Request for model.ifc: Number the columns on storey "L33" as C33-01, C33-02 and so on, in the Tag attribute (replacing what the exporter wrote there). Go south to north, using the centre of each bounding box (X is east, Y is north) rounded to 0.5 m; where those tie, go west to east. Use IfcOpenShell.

First a look at what the model holds.

```python
import ifcopenshell
import ifcopenshell.util.element
import ifcopenshell.util.placement

model = ifcopenshell.open("model.ifc")
print(model.schema)
storey = next(s for s in model.by_type("IfcBuildingStorey") if s.Name == "L33")
columns = [e for e in ifcopenshell.util.element.get_decomposition(storey) if e.is_a("IfcColumn")]
for e in sorted(columns, key=lambda e: e.id()):
    origin = ifcopenshell.util.placement.get_local_placement(e.ObjectPlacement)[:3, 3]
    print(e.id(), e.Tag, e.Name, origin.round(2) + 0.0, sep=" | ")
```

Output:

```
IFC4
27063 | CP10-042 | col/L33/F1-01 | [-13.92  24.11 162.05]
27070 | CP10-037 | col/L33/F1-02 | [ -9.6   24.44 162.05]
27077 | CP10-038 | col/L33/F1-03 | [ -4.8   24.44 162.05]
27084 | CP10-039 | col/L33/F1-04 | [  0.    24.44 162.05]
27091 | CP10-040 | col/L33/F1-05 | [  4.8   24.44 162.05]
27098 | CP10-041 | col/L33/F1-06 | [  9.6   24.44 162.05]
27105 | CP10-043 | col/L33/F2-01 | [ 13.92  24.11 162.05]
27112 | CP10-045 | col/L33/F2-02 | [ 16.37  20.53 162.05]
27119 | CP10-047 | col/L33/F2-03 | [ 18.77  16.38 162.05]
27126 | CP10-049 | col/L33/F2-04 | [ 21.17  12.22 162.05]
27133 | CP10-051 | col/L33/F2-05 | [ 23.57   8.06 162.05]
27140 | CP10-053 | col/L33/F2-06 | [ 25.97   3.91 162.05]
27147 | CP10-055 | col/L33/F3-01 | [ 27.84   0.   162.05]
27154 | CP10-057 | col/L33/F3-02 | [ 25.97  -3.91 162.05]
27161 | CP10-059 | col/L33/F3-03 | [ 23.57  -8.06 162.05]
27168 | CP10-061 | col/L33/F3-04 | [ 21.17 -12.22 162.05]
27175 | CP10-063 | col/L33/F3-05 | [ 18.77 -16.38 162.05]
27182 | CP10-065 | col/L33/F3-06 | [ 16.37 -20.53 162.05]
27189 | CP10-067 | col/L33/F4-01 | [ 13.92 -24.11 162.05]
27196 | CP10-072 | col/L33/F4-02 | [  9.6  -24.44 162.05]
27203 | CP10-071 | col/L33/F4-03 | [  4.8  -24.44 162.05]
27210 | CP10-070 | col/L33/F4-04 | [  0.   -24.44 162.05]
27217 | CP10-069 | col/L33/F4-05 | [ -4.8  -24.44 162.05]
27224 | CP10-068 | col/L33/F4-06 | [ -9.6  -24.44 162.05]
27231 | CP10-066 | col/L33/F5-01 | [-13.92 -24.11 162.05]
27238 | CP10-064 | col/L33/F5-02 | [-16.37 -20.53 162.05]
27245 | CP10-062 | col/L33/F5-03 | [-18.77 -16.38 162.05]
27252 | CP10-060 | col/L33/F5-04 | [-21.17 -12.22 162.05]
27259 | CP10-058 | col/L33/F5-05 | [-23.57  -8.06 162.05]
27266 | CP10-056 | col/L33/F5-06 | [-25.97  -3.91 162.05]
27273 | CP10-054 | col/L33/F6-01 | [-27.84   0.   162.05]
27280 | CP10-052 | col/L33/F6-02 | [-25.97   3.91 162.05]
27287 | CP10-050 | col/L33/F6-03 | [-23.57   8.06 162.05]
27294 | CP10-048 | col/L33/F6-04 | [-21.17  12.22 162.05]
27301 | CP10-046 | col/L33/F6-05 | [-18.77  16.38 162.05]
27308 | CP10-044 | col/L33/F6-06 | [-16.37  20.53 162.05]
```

```python
import ifcopenshell
import ifcopenshell.geom
import ifcopenshell.util.element
import ifcopenshell.util.shape

model = ifcopenshell.open("model.ifc")
settings = ifcopenshell.geom.settings()
settings.set("use-world-coords", True)


def centre(element):
    shape = ifcopenshell.geom.create_shape(settings, element)
    return ifcopenshell.util.shape.get_bbox_centroid(shape.geometry)


storey = next(s for s in model.by_type("IfcBuildingStorey") if s.Name == "L33")
columns = [e for e in ifcopenshell.util.element.get_decomposition(storey) if e.is_a("IfcColumn")]

# Insertion points can sit at a corner or the storey origin, so sort by the geometry (in metres).
centres = {e: centre(e) for e in columns}
columns.sort(key=lambda e: (round(centres[e][1] / 0.5), centres[e][0]))

for i, e in enumerate(columns, start=1):
    number = f"C33-{i:02d}"
    e.Tag = number
    print(e.id(), number)

model.write("model-out.ifc")
```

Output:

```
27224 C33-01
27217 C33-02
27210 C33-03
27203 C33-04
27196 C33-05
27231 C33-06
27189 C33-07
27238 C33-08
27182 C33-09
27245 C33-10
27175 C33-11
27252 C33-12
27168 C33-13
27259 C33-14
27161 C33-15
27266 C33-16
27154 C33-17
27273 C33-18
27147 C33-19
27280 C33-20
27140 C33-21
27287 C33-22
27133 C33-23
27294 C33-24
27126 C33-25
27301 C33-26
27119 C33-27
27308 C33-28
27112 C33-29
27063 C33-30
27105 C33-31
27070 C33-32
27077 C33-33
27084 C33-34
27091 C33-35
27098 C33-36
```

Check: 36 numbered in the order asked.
